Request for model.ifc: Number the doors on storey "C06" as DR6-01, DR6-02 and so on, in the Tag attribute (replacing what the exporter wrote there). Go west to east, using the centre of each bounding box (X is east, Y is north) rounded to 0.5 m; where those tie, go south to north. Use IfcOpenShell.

First a look at what the model holds.

```python
import ifcopenshell
import ifcopenshell.util.element
import ifcopenshell.util.placement

model = ifcopenshell.open("model.ifc")
print(model.schema)
storey = next(s for s in model.by_type("IfcBuildingStorey") if s.Name == "C06")
doors = [e for e in ifcopenshell.util.element.get_decomposition(storey) if e.is_a("IfcDoor")]
for e in sorted(doors, key=lambda e: e.id()):
    origin = ifcopenshell.util.placement.get_local_placement(e.ObjectPlacement)[:3, 3]
    print(e.id(), e.Tag, e.Name, origin.round(2) + 0.0, sep=" | ")
```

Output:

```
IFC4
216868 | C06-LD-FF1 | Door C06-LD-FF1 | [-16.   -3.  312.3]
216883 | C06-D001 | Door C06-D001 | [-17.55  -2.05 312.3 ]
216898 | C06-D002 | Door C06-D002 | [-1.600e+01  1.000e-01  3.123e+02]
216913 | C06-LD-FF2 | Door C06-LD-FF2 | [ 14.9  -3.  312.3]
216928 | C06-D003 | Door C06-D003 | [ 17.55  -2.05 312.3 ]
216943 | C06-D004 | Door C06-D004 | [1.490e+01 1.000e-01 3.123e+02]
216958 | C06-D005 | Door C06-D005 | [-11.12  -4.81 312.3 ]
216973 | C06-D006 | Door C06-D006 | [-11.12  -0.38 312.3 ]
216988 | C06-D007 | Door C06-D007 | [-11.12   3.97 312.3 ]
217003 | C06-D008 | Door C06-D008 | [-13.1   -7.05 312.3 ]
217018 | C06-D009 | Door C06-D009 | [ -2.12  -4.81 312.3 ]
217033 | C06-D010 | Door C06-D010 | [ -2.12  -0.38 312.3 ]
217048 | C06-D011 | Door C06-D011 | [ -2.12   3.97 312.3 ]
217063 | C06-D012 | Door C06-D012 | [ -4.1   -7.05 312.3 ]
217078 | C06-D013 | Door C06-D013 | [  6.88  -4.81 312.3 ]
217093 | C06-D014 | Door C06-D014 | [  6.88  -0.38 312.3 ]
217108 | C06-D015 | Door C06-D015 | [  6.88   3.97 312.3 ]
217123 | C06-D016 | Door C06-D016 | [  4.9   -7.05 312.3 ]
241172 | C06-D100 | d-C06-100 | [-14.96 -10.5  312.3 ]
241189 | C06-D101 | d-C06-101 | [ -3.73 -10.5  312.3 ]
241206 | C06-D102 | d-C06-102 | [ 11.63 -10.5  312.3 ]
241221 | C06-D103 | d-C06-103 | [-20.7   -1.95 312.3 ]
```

```python
import ifcopenshell
import ifcopenshell.geom
import ifcopenshell.util.element
import ifcopenshell.util.shape

model = ifcopenshell.open("model.ifc")
settings = ifcopenshell.geom.settings()
settings.set("use-world-coords", True)


def centre(element):
    shape = ifcopenshell.geom.create_shape(settings, element)
    return ifcopenshell.util.shape.get_bbox_centroid(shape.geometry)


storey = next(s for s in model.by_type("IfcBuildingStorey") if s.Name == "C06")
doors = [e for e in ifcopenshell.util.element.get_decomposition(storey) if e.is_a("IfcDoor")]

# Insertion points can sit at a corner or the storey origin, so sort by the geometry (in metres).
centres = {e: centre(e) for e in doors}
doors.sort(key=lambda e: (round(centres[e][0] / 0.5), centres[e][1]))

for i, e in enumerate(doors, start=1):
    number = f"DR6-{i:02d}"
    e.Tag = number
    print(e.id(), number)

model.write("model_rev.ifc")
```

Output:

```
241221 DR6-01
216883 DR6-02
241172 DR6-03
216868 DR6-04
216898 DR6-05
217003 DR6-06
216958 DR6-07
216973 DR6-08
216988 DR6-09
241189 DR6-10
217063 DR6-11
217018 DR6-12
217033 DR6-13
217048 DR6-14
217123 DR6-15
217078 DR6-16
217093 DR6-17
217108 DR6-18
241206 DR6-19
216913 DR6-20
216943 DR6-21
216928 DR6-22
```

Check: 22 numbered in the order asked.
